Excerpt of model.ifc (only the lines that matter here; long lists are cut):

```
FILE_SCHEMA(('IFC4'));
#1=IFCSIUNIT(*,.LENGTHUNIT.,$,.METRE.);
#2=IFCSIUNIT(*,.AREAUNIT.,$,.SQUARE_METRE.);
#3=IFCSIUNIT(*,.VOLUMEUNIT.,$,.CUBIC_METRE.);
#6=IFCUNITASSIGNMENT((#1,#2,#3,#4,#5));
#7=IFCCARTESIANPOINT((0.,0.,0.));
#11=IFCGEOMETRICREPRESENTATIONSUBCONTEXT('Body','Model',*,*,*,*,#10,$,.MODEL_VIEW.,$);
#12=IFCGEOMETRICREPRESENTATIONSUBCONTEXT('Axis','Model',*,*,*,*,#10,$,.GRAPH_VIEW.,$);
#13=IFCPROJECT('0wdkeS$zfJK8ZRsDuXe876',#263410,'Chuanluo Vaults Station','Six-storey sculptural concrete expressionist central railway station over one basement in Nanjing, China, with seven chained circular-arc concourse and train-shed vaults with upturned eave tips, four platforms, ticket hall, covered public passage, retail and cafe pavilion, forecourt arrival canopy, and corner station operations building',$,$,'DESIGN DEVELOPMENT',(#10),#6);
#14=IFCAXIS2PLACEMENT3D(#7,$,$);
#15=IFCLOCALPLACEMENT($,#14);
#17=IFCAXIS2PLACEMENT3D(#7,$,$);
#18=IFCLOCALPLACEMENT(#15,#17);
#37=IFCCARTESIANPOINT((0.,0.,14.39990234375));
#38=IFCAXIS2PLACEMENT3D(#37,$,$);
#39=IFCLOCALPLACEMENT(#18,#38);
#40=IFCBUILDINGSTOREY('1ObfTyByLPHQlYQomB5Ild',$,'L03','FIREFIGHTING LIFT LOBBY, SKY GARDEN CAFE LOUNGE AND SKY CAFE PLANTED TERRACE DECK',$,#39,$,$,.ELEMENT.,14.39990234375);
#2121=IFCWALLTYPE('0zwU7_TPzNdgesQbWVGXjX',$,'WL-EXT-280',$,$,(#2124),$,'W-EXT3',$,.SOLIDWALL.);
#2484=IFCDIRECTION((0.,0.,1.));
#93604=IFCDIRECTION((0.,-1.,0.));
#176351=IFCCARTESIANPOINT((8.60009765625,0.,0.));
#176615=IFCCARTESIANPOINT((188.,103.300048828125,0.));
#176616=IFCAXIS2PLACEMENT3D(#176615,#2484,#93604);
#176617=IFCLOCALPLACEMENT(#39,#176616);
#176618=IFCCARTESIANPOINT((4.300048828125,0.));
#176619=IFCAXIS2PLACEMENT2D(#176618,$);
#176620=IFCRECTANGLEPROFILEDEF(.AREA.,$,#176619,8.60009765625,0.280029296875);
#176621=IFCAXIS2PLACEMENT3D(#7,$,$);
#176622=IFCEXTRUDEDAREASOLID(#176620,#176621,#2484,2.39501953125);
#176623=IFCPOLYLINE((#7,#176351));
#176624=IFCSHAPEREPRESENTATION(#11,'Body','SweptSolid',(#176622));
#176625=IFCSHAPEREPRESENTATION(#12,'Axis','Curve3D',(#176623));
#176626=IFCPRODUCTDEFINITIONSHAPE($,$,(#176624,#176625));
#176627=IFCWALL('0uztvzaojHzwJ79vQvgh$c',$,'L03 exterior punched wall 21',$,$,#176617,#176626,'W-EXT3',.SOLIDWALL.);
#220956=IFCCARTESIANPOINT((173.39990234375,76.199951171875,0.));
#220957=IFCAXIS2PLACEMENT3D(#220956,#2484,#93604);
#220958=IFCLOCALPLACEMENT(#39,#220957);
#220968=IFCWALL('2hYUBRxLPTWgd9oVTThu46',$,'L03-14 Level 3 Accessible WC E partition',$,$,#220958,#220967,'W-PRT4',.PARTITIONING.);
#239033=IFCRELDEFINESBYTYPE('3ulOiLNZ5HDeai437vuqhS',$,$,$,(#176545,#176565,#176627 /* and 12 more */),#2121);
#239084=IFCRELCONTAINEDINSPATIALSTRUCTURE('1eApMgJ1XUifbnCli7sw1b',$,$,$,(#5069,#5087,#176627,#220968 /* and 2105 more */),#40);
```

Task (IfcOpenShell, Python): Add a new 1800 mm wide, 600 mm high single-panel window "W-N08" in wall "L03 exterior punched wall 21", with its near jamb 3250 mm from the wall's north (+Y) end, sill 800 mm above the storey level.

```python
import numpy as np
import ifcopenshell
import ifcopenshell.api.feature
import ifcopenshell.api.geometry
import ifcopenshell.api.root
import ifcopenshell.api.spatial
import ifcopenshell.geom
import ifcopenshell.util.element
import ifcopenshell.util.placement
import ifcopenshell.util.representation
import ifcopenshell.util.shape
import ifcopenshell.util.unit

model = ifcopenshell.open("model.ifc")
unit_scale = ifcopenshell.util.unit.calculate_unit_scale(model)
settings = ifcopenshell.geom.settings()


def volume(element):
    """Net volume in cubic metres, openings subtracted."""
    shape = ifcopenshell.geom.create_shape(settings, element)
    return ifcopenshell.util.shape.get_volume(shape.geometry)


wall = model.by_guid("0uztvzaojHzwJ79vQvgh$c")
storey = ifcopenshell.util.element.get_container(wall, ifc_class="IfcBuildingStorey")
context = ifcopenshell.util.representation.get_context(model, "Model", "Body", "MODEL_VIEW")
before = volume(wall)

width, height, from_end, sill = 1.8, 0.6, 3.25, 0.8  # metres

# The wall runs along its own X axis, and the end named is its -X end.
wall_shape = ifcopenshell.geom.create_shape(settings, wall)
x, y, z = ifcopenshell.util.shape.get_vertices(wall_shape.geometry).T
start = x.min() + from_end
face, thickness = float(y.min()), float(y.max() - y.min())
wall_matrix = ifcopenshell.util.placement.get_local_placement(wall.ObjectPlacement)
level = ifcopenshell.util.placement.get_local_placement(storey.ObjectPlacement)[2, 3]


def in_wall(x, y):
    """Placement at x, y metres in the wall's axes, at sill height."""
    matrix = wall_matrix.copy()
    matrix[:, 3] = wall_matrix @ np.array([x / unit_scale, y / unit_scale, 0.0, 1.0])
    matrix[2, 3] = level + sill / unit_scale
    return matrix


# Opening: a box that overshoots both wall faces by 50 mm.
opening = ifcopenshell.api.root.create_entity(model, ifc_class="IfcOpeningElement", predefined_type="OPENING")
box = ifcopenshell.api.geometry.add_wall_representation(
    model, context=context, length=width, height=height, thickness=thickness + 0.1
)
ifcopenshell.api.geometry.assign_representation(model, product=opening, representation=box)
ifcopenshell.api.geometry.edit_object_placement(model, product=opening, matrix=in_wall(start, face - 0.05), is_si=False)
ifcopenshell.api.feature.add_feature(model, feature=opening, element=wall)

window = ifcopenshell.api.root.create_entity(model, ifc_class="IfcWindow", name="W-N08", predefined_type="WINDOW")
window.OverallWidth, window.OverallHeight = width / unit_scale, height / unit_scale
window.PartitioningType = "SINGLE_PANEL"
body = ifcopenshell.api.geometry.add_window_representation(
    model,
    context=context,
    overall_width=window.OverallWidth,
    overall_height=window.OverallHeight,
    partition_type="SINGLE_PANEL",
)
ifcopenshell.api.geometry.assign_representation(model, product=window, representation=body)
ifcopenshell.api.spatial.assign_container(model, products=[window], relating_structure=storey)
ifcopenshell.api.feature.add_filling(model, opening=opening, element=window)

# Centre the window in the wall's thickness.
ifcopenshell.api.geometry.edit_object_placement(model, product=window, matrix=in_wall(start, face), is_si=False)
window_shape = ifcopenshell.geom.create_shape(settings, window)
depth = ifcopenshell.util.shape.get_vertices(window_shape.geometry)[:, 1]
offset = face + thickness / 2 - (depth.min() + depth.max()) / 2
ifcopenshell.api.geometry.edit_object_placement(model, product=window, matrix=in_wall(start, offset), is_si=False)

after = volume(wall)

print(f"wall volume {before:.3f} -> {after:.3f} m3")

model.write("model_edited.ifc")
```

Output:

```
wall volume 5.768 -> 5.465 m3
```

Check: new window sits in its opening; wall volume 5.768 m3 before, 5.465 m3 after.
